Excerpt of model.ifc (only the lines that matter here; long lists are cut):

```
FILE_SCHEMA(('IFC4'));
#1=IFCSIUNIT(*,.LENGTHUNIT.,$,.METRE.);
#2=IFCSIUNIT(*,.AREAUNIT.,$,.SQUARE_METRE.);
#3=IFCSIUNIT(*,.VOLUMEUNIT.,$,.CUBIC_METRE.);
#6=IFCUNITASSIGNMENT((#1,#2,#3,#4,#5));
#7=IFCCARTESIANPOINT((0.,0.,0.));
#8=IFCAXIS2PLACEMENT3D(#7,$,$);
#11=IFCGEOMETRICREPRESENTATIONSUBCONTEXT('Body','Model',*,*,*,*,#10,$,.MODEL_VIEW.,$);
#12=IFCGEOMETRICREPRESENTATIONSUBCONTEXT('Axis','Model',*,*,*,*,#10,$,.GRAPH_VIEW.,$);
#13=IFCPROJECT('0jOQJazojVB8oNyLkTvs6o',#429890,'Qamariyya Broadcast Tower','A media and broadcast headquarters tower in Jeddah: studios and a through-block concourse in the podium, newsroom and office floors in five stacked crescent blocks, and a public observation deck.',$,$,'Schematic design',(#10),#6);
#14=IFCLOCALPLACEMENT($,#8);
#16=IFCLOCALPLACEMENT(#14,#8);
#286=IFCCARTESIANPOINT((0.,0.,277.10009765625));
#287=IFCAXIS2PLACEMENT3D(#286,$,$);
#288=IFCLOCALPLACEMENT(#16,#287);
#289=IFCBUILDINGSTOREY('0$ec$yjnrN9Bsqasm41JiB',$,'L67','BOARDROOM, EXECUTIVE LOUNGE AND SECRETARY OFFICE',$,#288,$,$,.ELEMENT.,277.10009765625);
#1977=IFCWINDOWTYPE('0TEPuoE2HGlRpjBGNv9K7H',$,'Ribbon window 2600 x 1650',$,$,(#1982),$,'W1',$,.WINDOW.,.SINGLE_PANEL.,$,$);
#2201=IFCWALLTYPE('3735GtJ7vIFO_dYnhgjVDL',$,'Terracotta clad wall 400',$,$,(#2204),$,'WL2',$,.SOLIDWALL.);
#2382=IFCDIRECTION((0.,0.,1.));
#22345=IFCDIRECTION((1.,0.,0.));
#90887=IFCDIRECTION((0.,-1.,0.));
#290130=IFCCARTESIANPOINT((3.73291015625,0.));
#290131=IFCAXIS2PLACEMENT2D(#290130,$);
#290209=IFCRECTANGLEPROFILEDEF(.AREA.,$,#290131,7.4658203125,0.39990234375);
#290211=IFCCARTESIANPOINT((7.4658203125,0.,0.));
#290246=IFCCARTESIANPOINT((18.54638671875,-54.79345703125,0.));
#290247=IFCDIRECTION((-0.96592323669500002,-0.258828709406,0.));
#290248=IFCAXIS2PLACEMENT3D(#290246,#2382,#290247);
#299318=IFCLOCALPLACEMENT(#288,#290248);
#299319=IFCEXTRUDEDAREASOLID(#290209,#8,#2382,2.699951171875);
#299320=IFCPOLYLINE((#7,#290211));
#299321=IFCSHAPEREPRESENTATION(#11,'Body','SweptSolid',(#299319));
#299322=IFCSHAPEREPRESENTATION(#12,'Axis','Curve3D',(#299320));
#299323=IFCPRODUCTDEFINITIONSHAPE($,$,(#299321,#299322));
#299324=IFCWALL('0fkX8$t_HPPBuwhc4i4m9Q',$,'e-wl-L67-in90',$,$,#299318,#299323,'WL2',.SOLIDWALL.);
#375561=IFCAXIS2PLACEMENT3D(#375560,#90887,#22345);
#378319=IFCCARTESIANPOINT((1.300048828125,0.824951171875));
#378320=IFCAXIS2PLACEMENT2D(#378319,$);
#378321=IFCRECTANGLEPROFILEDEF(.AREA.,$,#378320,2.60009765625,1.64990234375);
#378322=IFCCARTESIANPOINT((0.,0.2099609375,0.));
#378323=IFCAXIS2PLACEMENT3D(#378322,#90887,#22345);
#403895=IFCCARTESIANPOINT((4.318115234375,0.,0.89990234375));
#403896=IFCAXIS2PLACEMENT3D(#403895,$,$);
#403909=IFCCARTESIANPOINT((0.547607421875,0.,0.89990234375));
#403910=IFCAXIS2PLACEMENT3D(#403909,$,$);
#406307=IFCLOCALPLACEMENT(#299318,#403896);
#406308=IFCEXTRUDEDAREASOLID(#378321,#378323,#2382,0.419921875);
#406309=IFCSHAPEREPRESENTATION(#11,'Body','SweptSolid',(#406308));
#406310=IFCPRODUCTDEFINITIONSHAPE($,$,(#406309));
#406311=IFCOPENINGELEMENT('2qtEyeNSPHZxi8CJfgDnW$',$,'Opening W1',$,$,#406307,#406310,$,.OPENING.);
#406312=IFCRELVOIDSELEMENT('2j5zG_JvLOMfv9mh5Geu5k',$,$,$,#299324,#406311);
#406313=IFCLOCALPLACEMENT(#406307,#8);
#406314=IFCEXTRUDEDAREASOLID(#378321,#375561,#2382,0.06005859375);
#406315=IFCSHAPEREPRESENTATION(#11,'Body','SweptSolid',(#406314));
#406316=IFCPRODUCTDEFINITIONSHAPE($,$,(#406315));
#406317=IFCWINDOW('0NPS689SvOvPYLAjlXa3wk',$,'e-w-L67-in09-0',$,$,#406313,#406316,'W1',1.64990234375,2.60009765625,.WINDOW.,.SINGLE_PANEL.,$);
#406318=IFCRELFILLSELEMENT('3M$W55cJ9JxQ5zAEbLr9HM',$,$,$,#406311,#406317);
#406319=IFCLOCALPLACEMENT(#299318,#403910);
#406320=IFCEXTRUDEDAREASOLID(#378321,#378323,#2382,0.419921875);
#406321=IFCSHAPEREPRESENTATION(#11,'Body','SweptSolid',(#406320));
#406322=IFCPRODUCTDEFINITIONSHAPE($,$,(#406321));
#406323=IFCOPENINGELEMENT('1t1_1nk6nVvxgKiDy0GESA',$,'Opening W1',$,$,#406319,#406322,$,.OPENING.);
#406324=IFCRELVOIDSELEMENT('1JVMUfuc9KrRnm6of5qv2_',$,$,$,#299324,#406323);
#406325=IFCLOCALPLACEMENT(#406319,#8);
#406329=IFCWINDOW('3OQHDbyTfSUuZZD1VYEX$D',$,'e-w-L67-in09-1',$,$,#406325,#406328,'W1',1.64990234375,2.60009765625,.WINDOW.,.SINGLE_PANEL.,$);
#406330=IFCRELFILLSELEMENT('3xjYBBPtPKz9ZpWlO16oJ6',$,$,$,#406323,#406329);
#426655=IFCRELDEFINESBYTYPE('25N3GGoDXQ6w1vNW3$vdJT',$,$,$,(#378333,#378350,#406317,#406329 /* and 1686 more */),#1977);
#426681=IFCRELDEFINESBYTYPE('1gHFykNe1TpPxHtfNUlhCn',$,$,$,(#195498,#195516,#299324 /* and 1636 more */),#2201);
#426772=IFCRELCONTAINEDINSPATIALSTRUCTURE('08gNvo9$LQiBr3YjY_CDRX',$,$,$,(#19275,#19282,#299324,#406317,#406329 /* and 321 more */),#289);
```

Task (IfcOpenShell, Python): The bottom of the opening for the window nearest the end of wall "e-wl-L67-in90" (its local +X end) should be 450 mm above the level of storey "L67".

```python
import numpy as np
import ifcopenshell
import ifcopenshell.api.geometry
import ifcopenshell.geom
import ifcopenshell.util.element
import ifcopenshell.util.placement
import ifcopenshell.util.shape
import ifcopenshell.util.unit

model = ifcopenshell.open("model.ifc")
unit_scale = ifcopenshell.util.unit.calculate_unit_scale(model)

window = model.by_guid("0NPS689SvOvPYLAjlXa3wk")
opening = window.FillsVoids[0].RelatingOpeningElement
storey = ifcopenshell.util.element.get_container(window, ifc_class="IfcBuildingStorey")
level = ifcopenshell.util.placement.get_local_placement(storey.ObjectPlacement)[2, 3]

# The opening's origin need not be at the sill, so measure its lowest point.
shape = ifcopenshell.geom.create_shape(ifcopenshell.geom.settings(), opening)
bottom = ifcopenshell.util.shape.get_shape_bottom_elevation(shape, shape.geometry) / unit_scale
dz = level + 0.45 / unit_scale - bottom

shift = np.array([0.0, 0.0, dz])
# The window is placed relative to its opening, so it follows when the opening moves.
matrix = ifcopenshell.util.placement.get_local_placement(opening.ObjectPlacement)
matrix[:3, 3] += shift
ifcopenshell.api.geometry.edit_object_placement(
    model, product=opening, matrix=matrix, is_si=False, should_transform_children=True
)

print(f"moved by {dz * unit_scale:+.3f} m")

model.write("model_edited.ifc")
```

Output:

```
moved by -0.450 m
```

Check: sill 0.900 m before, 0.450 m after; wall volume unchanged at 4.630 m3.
